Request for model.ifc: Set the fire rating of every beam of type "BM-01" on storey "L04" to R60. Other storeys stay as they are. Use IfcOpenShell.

First a look at what the model holds.

```python
import ifcopenshell
import ifcopenshell.util.element

model = ifcopenshell.open("model.ifc")
print(model.schema)
storey = next(s for s in model.by_type("IfcBuildingStorey") if s.Name == "L04")
beams = [e for e in ifcopenshell.util.element.get_decomposition(storey) if e.is_a("IfcBeam")]
seen = {}
for e in beams:
    element_type = ifcopenshell.util.element.get_type(e)
    key = (element_type.Name if element_type != e and element_type else None, ifcopenshell.util.element.get_pset(e, "Pset_BeamCommon", "FireRating"))
    seen[key] = seen.get(key, 0) + 1
for (name, value), count in sorted(seen.items(), key=str):
    print(count, "x", name, "|", value)
```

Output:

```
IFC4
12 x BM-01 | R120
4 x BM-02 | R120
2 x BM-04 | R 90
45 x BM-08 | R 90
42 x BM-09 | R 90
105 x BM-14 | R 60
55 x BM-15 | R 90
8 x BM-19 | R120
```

```python
import ifcopenshell
import ifcopenshell.api.pset
import ifcopenshell.util.element

model = ifcopenshell.open("model.ifc")

storey = next(s for s in model.by_type("IfcBuildingStorey") if s.Name == "L04")
beams = [e for e in ifcopenshell.util.element.get_decomposition(storey) if e.is_a("IfcBeam")]

count = 0
for e in beams:
    element_type = ifcopenshell.util.element.get_type(e)
    if element_type in (None, e) or element_type.Name != "BM-01":
        continue
    # add_pset returns the element's existing set when there is one.
    pset = ifcopenshell.api.pset.add_pset(model, product=e, name="Pset_BeamCommon")
    ifcopenshell.api.pset.edit_pset(model, pset=pset, properties={"FireRating": "R60"})
    count += 1

print(count, "beams updated")

model.write("model_v2.ifc")
```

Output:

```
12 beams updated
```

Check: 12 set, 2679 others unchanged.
